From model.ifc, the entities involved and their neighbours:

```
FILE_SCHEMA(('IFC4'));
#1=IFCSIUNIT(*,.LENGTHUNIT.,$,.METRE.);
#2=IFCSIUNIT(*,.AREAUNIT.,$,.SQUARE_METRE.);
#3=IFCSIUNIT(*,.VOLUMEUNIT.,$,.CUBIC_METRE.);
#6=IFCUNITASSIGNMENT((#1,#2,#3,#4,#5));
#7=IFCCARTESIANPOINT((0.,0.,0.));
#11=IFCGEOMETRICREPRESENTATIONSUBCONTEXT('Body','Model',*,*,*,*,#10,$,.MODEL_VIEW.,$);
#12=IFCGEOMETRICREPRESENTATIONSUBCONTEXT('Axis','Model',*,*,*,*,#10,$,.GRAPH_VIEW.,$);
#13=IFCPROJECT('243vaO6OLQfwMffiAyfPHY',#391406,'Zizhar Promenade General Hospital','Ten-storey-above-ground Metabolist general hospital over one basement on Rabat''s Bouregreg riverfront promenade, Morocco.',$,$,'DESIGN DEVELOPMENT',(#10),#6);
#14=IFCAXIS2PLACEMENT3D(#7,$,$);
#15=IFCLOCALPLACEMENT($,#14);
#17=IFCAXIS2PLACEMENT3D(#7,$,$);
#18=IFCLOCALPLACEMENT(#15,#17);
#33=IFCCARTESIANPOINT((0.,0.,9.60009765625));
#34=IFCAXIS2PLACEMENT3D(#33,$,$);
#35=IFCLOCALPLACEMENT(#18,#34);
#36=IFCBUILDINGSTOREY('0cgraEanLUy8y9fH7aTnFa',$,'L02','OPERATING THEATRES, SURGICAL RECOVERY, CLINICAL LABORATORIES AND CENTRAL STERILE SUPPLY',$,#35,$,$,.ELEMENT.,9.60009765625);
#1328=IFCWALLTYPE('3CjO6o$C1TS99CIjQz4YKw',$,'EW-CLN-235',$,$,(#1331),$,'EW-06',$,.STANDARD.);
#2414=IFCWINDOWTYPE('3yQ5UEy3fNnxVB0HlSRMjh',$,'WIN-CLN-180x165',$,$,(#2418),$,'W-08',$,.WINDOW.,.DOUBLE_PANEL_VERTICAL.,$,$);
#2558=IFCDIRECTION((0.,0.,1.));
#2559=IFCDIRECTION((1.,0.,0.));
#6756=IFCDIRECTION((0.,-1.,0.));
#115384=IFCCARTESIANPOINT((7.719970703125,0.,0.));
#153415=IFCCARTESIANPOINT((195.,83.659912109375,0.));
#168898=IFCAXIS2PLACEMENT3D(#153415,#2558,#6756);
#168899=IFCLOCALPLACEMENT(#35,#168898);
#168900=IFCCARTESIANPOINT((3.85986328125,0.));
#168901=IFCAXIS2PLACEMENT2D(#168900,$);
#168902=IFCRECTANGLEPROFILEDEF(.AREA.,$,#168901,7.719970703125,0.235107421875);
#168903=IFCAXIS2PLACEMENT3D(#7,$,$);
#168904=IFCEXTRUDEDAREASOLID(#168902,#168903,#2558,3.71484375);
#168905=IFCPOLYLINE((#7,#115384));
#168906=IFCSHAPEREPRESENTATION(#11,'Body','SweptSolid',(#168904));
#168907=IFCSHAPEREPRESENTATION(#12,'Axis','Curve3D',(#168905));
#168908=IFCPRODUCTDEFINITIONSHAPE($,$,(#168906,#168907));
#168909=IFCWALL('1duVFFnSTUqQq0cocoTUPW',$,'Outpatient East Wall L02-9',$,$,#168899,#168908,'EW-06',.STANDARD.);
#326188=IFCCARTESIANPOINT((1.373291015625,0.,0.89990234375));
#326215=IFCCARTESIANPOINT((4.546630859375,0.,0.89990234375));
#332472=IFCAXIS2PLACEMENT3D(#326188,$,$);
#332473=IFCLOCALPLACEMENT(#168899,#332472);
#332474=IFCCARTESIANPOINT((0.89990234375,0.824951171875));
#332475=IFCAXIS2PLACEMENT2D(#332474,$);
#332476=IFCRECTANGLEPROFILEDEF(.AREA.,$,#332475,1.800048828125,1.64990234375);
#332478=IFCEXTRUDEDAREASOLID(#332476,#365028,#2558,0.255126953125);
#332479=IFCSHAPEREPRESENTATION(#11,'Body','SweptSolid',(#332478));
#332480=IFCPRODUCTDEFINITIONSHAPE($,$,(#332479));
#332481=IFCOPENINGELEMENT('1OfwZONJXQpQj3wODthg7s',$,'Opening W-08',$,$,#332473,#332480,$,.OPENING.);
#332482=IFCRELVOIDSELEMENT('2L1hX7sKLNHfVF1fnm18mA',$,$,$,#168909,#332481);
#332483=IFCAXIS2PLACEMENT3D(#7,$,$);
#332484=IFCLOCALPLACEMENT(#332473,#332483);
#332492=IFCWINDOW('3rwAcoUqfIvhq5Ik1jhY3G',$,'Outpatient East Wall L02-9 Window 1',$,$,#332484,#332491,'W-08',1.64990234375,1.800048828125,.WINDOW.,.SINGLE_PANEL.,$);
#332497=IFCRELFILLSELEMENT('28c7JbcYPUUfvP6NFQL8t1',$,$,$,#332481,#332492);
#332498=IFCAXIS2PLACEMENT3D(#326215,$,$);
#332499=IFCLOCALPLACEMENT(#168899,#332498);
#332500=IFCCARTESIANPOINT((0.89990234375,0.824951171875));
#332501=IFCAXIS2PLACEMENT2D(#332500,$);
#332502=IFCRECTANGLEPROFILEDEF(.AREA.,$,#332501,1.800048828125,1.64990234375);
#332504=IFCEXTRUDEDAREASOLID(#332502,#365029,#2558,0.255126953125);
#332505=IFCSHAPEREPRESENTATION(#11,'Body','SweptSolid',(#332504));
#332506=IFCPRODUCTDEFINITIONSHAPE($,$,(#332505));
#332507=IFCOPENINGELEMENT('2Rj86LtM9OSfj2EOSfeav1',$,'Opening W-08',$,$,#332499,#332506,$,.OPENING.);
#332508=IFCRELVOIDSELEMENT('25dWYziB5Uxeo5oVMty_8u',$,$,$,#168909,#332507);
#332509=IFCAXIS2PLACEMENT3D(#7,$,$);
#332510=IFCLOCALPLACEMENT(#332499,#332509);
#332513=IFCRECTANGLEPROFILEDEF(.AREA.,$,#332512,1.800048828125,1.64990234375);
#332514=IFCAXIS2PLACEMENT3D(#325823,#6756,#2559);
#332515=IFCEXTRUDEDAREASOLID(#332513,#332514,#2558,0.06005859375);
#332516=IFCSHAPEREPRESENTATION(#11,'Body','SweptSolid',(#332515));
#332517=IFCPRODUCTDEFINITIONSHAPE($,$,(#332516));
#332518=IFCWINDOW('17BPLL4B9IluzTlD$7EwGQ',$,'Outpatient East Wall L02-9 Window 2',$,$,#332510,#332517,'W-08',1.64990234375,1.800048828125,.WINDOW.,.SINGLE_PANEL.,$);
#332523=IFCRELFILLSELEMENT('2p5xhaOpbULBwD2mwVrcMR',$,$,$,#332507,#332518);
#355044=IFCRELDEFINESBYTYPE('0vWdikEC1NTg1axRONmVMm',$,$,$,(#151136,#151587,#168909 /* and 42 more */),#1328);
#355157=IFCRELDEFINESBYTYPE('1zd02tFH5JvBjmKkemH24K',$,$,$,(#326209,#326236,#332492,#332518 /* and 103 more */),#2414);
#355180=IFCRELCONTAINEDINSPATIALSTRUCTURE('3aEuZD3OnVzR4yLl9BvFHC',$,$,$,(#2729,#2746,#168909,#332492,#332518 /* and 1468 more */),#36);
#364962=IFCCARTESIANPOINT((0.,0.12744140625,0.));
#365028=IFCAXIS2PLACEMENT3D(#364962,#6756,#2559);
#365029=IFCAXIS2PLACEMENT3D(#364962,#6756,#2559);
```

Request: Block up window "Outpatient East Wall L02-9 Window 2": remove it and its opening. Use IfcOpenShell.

```python
import ifcopenshell
import ifcopenshell.api.feature
import ifcopenshell.api.root
import ifcopenshell.geom
import ifcopenshell.util.shape

model = ifcopenshell.open("model.ifc")
settings = ifcopenshell.geom.settings()


def volume(element):
    """Net volume in cubic metres, openings subtracted."""
    shape = ifcopenshell.geom.create_shape(settings, element)
    return ifcopenshell.util.shape.get_volume(shape.geometry)


window = model.by_guid("17BPLL4B9IluzTlD$7EwGQ")
opening = window.FillsVoids[0].RelatingOpeningElement
wall = opening.VoidsElements[0].RelatingBuildingElement
before = volume(wall)

ifcopenshell.api.root.remove_product(model, product=window)
ifcopenshell.api.feature.remove_feature(model, feature=opening)

after = volume(wall)

print(f"wall volume {before:.3f} -> {after:.3f} m3")

model.write("model_edited.ifc")
```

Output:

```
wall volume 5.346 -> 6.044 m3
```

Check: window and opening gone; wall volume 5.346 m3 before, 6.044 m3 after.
